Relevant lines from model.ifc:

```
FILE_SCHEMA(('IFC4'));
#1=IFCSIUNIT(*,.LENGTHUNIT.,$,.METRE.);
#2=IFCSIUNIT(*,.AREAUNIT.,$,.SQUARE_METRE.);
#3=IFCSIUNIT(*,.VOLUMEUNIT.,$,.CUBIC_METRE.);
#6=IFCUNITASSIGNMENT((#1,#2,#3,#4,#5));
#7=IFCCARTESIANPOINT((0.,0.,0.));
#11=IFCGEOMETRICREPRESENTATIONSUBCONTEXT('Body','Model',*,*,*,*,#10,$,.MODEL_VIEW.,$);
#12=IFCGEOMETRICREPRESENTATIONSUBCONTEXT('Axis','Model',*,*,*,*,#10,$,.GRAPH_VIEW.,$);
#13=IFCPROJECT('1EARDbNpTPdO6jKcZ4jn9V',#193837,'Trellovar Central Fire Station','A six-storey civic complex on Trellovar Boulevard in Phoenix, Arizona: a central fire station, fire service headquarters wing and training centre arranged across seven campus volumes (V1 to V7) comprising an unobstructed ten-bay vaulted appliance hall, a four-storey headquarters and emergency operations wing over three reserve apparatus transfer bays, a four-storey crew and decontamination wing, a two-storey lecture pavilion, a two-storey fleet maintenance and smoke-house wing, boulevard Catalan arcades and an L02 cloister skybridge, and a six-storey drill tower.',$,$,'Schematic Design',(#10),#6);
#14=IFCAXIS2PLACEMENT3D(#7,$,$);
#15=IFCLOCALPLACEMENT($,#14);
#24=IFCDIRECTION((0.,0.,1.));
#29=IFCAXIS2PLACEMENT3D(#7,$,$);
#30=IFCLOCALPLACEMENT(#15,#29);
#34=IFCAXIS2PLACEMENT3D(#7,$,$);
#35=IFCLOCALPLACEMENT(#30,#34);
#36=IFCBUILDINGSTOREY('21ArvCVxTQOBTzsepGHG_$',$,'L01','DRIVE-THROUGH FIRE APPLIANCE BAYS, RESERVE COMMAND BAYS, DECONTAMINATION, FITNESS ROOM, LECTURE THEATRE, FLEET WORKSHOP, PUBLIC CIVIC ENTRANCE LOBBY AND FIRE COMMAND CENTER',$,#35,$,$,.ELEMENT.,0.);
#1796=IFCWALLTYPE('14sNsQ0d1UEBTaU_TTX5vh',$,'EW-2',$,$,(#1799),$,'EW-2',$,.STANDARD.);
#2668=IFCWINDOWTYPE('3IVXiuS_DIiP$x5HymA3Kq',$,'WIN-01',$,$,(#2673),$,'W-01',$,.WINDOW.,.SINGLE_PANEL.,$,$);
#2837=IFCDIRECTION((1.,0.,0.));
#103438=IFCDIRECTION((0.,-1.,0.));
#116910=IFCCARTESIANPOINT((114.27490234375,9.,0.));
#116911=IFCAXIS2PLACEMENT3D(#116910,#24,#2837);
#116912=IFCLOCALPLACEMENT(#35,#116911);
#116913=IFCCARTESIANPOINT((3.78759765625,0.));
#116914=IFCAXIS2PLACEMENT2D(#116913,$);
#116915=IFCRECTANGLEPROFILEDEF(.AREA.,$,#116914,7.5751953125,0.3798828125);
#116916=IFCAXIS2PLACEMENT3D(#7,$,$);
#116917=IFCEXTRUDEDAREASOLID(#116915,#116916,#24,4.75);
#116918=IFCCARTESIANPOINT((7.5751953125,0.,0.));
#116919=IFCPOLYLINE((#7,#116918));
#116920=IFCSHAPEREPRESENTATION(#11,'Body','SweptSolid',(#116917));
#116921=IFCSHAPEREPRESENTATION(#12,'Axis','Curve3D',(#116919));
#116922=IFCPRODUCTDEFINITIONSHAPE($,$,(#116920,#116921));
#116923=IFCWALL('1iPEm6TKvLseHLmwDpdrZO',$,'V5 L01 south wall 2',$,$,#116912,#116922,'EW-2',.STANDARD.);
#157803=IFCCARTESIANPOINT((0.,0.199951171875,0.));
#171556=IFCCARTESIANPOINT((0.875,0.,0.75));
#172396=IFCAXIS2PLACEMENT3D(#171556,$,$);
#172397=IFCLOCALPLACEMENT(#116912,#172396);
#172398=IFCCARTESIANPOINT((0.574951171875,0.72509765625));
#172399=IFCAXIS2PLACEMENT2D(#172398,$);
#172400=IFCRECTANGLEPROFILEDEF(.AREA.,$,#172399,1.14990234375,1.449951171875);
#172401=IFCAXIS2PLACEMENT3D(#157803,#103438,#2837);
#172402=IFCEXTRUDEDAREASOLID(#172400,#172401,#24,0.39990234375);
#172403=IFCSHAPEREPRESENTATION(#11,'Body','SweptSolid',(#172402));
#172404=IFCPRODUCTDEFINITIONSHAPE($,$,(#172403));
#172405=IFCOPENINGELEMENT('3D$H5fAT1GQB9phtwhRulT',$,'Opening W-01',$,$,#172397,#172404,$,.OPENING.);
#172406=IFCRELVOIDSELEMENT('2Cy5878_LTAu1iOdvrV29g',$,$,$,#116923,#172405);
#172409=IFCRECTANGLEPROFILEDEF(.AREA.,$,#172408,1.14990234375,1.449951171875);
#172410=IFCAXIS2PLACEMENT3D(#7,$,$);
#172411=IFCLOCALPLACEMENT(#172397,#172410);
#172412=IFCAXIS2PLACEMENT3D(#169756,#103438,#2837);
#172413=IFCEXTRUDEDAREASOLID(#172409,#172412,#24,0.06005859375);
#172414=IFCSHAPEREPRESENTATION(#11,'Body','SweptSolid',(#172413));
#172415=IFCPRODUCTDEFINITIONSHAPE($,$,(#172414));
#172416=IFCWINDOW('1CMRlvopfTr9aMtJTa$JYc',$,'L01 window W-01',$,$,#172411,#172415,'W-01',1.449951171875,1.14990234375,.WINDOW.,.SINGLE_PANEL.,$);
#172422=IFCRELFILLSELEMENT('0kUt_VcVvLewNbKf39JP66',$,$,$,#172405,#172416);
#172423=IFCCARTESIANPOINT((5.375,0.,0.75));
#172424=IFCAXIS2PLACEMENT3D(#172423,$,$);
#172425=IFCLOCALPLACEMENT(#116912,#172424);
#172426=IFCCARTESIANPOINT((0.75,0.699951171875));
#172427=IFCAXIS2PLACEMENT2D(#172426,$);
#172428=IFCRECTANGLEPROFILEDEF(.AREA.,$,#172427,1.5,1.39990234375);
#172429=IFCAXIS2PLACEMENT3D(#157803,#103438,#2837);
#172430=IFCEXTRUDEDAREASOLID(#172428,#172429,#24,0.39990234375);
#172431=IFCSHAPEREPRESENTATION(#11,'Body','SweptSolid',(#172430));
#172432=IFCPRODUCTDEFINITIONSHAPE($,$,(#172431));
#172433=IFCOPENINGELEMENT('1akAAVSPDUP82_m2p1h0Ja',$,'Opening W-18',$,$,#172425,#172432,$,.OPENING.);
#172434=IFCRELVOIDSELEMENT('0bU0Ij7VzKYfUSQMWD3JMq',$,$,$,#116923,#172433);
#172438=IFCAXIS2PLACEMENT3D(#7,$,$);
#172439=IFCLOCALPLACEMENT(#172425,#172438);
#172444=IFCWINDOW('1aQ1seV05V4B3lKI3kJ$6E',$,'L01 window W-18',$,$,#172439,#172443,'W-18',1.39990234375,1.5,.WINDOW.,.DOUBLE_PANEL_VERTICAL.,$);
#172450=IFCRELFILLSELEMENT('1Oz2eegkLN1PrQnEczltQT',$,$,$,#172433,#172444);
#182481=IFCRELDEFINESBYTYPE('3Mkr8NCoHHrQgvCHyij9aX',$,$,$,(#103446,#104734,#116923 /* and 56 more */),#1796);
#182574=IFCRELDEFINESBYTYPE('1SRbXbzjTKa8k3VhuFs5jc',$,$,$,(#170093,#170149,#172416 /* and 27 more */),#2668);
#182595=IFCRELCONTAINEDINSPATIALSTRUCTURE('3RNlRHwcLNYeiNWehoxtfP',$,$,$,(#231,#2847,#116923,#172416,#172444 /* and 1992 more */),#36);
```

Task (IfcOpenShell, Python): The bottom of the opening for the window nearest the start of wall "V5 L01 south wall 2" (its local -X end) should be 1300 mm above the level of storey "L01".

```python
import numpy as np
import ifcopenshell
import ifcopenshell.api.geometry
import ifcopenshell.geom
import ifcopenshell.util.element
import ifcopenshell.util.placement
import ifcopenshell.util.shape
import ifcopenshell.util.unit

model = ifcopenshell.open("model.ifc")
unit_scale = ifcopenshell.util.unit.calculate_unit_scale(model)

window = model.by_guid("1CMRlvopfTr9aMtJTa$JYc")
opening = window.FillsVoids[0].RelatingOpeningElement
storey = ifcopenshell.util.element.get_container(window, ifc_class="IfcBuildingStorey")
level = ifcopenshell.util.placement.get_local_placement(storey.ObjectPlacement)[2, 3]

# The opening's origin need not be at the sill, so measure its lowest point.
shape = ifcopenshell.geom.create_shape(ifcopenshell.geom.settings(), opening)
bottom = ifcopenshell.util.shape.get_shape_bottom_elevation(shape, shape.geometry) / unit_scale
dz = level + 1.3 / unit_scale - bottom

shift = np.array([0.0, 0.0, dz])
# The window is placed relative to its opening, so it follows when the opening moves.
matrix = ifcopenshell.util.placement.get_local_placement(opening.ObjectPlacement)
matrix[:3, 3] += shift
ifcopenshell.api.geometry.edit_object_placement(
    model, product=opening, matrix=matrix, is_si=False, should_transform_children=True
)

print(f"moved by {dz * unit_scale:+.3f} m")

model.write("model_rev.ifc")
```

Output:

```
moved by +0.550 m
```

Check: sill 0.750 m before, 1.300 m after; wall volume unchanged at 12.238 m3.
